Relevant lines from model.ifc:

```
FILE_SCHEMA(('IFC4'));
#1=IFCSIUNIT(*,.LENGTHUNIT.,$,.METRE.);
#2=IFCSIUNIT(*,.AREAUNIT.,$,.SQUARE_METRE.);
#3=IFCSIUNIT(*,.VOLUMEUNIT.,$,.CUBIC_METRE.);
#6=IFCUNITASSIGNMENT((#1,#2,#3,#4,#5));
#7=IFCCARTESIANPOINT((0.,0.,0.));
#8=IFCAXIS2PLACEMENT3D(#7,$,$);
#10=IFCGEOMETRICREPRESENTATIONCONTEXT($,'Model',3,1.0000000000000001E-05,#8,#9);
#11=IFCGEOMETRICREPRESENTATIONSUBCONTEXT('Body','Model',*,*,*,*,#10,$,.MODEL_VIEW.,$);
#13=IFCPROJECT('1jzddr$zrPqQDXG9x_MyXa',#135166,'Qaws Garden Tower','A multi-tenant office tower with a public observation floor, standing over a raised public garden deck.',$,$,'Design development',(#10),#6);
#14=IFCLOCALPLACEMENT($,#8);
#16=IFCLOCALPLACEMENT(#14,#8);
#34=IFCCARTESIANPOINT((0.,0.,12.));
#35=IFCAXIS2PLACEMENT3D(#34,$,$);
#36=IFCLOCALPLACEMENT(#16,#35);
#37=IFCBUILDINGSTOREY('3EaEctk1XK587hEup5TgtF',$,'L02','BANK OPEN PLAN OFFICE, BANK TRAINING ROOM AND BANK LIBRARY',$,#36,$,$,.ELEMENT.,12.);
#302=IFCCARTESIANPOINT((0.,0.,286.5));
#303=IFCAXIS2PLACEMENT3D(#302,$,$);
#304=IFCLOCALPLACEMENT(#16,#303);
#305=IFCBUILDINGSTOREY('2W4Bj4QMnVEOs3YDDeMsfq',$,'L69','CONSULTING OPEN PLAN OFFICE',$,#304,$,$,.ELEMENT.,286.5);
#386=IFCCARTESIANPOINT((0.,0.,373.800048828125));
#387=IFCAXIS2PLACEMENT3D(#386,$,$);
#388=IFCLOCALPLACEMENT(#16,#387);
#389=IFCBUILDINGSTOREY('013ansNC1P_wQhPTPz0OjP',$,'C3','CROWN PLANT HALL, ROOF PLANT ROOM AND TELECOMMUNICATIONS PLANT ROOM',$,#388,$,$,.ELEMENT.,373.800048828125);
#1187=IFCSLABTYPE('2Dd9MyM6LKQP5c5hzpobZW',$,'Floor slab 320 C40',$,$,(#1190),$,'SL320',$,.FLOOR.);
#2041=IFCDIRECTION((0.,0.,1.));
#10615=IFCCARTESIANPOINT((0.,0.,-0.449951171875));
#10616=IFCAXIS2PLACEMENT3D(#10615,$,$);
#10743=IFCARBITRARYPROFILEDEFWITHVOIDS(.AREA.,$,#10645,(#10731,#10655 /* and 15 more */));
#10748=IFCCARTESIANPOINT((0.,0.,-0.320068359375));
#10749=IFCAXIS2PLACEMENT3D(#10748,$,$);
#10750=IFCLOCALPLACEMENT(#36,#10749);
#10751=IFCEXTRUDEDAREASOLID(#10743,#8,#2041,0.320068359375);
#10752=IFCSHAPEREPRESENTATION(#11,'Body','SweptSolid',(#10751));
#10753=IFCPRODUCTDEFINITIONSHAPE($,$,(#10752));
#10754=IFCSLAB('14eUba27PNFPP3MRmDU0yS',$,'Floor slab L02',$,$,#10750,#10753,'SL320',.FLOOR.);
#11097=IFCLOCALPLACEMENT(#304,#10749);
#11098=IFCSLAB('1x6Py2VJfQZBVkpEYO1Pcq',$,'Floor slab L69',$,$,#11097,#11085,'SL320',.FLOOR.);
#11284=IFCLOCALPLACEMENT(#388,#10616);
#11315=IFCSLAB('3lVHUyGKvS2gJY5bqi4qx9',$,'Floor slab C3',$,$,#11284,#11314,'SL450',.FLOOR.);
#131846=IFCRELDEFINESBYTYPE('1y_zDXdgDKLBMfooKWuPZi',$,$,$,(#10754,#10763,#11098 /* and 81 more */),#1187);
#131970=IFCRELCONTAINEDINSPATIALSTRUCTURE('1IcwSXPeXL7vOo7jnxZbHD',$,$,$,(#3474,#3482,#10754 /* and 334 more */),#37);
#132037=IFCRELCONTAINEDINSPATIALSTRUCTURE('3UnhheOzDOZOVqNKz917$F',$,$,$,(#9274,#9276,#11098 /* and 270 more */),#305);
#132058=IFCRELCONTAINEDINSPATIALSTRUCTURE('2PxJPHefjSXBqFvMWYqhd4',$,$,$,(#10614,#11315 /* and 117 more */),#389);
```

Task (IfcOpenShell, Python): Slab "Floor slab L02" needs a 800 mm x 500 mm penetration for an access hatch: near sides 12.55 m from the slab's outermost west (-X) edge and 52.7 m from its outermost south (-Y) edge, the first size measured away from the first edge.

```python
import numpy as np
import ifcopenshell
import ifcopenshell.api.feature
import ifcopenshell.api.geometry
import ifcopenshell.api.root
import ifcopenshell.geom
import ifcopenshell.util.placement
import ifcopenshell.util.representation
import ifcopenshell.util.shape
import ifcopenshell.util.unit

model = ifcopenshell.open("model.ifc")
unit_scale = ifcopenshell.util.unit.calculate_unit_scale(model)
settings = ifcopenshell.geom.settings()


def volume(element):
    """Net volume in cubic metres, openings subtracted."""
    shape = ifcopenshell.geom.create_shape(settings, element)
    return ifcopenshell.util.shape.get_volume(shape.geometry)


slab = model.by_guid("14eUba27PNFPP3MRmDU0yS")
before = volume(slab)

# Extent in the slab's own axes, in metres. The edges named are its -X and -Y sides.
slab_shape = ifcopenshell.geom.create_shape(settings, slab)
vertices = ifcopenshell.util.shape.get_vertices(slab_shape.geometry)
x_min, y_min, bottom = vertices.min(axis=0)
top = vertices[:, 2].max()

opening = ifcopenshell.api.root.create_entity(model, ifc_class="IfcOpeningElement", name="Access hatch opening", predefined_type="OPENING")
context = ifcopenshell.util.representation.get_context(model, "Model", "Body", "MODEL_VIEW")
width, depth = 0.8, 0.5
outline = [(0.0, 0.0), (width, 0.0), (width, depth), (0.0, depth), (0.0, 0.0)]
# Overshoot both faces by 50 mm so the cut is clean.
shape = ifcopenshell.api.geometry.add_slab_representation(
    model, context=context, depth=top - bottom + 0.1, polyline=outline
)
ifcopenshell.api.geometry.assign_representation(model, product=opening, representation=shape)

matrix = ifcopenshell.util.placement.get_local_placement(slab.ObjectPlacement)
matrix[:, 3] = matrix @ np.append(np.array([x_min + 12.55, y_min + 52.7, bottom - 0.05]) / unit_scale, 1.0)
ifcopenshell.api.geometry.edit_object_placement(model, product=opening, matrix=matrix, is_si=False)
ifcopenshell.api.feature.add_feature(model, feature=opening, element=slab)

after = volume(slab)

print(f"slab volume {before:.3f} -> {after:.3f} m3")

model.write("model_rev.ifc")
```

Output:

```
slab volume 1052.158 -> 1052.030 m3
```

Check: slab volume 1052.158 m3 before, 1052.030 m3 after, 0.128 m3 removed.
